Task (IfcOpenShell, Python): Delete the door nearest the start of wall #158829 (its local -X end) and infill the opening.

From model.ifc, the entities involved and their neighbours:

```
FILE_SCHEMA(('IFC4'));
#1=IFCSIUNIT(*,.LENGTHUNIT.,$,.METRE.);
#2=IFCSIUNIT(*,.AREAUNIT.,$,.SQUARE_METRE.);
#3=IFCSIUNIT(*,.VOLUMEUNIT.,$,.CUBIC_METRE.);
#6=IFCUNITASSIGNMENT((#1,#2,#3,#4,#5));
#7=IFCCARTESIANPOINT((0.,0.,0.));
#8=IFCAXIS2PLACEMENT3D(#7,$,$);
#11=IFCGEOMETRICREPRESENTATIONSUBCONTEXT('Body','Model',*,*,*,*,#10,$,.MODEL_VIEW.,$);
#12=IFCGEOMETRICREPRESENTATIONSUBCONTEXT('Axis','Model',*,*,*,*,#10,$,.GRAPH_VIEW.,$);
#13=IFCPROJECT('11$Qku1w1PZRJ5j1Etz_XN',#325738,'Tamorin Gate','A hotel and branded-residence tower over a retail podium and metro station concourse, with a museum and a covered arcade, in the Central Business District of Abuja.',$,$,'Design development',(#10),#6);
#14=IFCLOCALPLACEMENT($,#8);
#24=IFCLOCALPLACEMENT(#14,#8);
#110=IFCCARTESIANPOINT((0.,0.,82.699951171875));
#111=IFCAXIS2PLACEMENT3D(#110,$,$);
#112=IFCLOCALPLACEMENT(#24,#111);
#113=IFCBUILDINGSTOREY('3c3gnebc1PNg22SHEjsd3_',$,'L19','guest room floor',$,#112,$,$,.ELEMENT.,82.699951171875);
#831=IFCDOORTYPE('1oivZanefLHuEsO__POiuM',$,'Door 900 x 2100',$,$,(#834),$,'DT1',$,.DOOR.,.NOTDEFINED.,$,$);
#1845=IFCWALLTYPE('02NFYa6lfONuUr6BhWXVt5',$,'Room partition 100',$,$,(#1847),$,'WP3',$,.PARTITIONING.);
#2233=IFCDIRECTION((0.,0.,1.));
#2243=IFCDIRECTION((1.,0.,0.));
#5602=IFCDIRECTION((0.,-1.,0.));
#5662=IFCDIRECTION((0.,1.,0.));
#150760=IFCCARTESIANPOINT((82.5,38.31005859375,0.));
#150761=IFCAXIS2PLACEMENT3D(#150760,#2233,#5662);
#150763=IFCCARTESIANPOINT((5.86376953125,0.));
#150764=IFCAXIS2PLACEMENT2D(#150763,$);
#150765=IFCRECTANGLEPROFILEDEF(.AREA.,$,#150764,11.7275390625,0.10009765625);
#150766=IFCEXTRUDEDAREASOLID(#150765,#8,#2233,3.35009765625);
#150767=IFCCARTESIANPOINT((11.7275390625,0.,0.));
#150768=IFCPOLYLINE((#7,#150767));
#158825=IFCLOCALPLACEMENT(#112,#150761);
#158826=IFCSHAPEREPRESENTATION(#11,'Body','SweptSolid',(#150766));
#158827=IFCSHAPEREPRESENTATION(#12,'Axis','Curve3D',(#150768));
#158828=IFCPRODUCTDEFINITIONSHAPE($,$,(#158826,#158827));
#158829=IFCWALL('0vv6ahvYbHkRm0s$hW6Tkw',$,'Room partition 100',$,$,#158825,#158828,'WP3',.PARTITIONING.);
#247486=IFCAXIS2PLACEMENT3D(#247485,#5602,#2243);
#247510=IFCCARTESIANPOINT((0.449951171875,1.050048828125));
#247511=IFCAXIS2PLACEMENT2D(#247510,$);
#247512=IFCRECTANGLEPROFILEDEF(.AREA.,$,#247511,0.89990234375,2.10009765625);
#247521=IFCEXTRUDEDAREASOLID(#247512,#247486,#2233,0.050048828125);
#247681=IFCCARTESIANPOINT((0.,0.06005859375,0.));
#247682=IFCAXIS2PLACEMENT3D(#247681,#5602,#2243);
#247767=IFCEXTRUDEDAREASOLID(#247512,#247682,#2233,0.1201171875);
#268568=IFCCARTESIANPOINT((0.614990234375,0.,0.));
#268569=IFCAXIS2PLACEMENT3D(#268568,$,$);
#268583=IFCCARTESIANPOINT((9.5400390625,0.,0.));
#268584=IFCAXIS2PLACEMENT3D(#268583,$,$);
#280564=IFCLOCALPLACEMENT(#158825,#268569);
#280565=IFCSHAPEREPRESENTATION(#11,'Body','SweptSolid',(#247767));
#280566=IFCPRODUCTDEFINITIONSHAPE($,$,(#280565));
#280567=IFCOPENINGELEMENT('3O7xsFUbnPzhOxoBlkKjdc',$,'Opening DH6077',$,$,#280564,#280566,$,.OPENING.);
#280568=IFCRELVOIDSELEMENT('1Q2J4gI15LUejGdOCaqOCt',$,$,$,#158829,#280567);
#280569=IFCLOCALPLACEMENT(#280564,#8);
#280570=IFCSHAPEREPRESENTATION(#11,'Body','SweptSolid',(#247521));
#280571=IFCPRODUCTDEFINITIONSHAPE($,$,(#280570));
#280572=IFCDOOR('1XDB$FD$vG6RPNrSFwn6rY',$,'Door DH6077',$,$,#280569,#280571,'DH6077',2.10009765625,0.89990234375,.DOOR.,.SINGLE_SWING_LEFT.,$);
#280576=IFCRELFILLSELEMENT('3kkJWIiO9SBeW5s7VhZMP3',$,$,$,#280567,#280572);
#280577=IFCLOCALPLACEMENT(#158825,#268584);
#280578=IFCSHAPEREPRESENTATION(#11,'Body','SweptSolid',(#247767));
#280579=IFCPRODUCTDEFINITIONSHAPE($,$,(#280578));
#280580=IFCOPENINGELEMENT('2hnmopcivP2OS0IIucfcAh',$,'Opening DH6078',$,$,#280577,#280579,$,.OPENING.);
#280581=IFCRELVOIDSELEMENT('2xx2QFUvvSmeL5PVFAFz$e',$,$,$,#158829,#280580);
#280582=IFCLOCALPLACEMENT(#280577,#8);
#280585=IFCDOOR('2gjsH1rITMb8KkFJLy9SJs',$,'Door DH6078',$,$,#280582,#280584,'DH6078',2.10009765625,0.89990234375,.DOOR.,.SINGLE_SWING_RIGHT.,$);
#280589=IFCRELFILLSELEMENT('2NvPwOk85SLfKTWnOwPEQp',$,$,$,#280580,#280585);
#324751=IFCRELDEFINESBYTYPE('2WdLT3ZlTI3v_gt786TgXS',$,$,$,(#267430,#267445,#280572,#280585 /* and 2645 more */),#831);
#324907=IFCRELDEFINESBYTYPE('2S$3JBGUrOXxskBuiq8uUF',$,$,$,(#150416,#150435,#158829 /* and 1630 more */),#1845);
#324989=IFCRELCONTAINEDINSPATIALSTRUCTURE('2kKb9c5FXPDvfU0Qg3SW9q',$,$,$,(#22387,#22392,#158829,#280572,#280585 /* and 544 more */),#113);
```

```python
import ifcopenshell
import ifcopenshell.api.feature
import ifcopenshell.api.root
import ifcopenshell.geom
import ifcopenshell.util.shape

model = ifcopenshell.open("model.ifc")
settings = ifcopenshell.geom.settings()


def volume(element):
    """Net volume in cubic metres, openings subtracted."""
    shape = ifcopenshell.geom.create_shape(settings, element)
    return ifcopenshell.util.shape.get_volume(shape.geometry)


door = model.by_guid("1XDB$FD$vG6RPNrSFwn6rY")
opening = door.FillsVoids[0].RelatingOpeningElement
wall = opening.VoidsElements[0].RelatingBuildingElement
before = volume(wall)

ifcopenshell.api.root.remove_product(model, product=door)
ifcopenshell.api.feature.remove_feature(model, feature=opening)

after = volume(wall)

print(f"wall volume {before:.3f} -> {after:.3f} m3")

model.write("model_v2.ifc")
```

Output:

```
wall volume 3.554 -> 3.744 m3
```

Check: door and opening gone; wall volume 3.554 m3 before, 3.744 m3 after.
